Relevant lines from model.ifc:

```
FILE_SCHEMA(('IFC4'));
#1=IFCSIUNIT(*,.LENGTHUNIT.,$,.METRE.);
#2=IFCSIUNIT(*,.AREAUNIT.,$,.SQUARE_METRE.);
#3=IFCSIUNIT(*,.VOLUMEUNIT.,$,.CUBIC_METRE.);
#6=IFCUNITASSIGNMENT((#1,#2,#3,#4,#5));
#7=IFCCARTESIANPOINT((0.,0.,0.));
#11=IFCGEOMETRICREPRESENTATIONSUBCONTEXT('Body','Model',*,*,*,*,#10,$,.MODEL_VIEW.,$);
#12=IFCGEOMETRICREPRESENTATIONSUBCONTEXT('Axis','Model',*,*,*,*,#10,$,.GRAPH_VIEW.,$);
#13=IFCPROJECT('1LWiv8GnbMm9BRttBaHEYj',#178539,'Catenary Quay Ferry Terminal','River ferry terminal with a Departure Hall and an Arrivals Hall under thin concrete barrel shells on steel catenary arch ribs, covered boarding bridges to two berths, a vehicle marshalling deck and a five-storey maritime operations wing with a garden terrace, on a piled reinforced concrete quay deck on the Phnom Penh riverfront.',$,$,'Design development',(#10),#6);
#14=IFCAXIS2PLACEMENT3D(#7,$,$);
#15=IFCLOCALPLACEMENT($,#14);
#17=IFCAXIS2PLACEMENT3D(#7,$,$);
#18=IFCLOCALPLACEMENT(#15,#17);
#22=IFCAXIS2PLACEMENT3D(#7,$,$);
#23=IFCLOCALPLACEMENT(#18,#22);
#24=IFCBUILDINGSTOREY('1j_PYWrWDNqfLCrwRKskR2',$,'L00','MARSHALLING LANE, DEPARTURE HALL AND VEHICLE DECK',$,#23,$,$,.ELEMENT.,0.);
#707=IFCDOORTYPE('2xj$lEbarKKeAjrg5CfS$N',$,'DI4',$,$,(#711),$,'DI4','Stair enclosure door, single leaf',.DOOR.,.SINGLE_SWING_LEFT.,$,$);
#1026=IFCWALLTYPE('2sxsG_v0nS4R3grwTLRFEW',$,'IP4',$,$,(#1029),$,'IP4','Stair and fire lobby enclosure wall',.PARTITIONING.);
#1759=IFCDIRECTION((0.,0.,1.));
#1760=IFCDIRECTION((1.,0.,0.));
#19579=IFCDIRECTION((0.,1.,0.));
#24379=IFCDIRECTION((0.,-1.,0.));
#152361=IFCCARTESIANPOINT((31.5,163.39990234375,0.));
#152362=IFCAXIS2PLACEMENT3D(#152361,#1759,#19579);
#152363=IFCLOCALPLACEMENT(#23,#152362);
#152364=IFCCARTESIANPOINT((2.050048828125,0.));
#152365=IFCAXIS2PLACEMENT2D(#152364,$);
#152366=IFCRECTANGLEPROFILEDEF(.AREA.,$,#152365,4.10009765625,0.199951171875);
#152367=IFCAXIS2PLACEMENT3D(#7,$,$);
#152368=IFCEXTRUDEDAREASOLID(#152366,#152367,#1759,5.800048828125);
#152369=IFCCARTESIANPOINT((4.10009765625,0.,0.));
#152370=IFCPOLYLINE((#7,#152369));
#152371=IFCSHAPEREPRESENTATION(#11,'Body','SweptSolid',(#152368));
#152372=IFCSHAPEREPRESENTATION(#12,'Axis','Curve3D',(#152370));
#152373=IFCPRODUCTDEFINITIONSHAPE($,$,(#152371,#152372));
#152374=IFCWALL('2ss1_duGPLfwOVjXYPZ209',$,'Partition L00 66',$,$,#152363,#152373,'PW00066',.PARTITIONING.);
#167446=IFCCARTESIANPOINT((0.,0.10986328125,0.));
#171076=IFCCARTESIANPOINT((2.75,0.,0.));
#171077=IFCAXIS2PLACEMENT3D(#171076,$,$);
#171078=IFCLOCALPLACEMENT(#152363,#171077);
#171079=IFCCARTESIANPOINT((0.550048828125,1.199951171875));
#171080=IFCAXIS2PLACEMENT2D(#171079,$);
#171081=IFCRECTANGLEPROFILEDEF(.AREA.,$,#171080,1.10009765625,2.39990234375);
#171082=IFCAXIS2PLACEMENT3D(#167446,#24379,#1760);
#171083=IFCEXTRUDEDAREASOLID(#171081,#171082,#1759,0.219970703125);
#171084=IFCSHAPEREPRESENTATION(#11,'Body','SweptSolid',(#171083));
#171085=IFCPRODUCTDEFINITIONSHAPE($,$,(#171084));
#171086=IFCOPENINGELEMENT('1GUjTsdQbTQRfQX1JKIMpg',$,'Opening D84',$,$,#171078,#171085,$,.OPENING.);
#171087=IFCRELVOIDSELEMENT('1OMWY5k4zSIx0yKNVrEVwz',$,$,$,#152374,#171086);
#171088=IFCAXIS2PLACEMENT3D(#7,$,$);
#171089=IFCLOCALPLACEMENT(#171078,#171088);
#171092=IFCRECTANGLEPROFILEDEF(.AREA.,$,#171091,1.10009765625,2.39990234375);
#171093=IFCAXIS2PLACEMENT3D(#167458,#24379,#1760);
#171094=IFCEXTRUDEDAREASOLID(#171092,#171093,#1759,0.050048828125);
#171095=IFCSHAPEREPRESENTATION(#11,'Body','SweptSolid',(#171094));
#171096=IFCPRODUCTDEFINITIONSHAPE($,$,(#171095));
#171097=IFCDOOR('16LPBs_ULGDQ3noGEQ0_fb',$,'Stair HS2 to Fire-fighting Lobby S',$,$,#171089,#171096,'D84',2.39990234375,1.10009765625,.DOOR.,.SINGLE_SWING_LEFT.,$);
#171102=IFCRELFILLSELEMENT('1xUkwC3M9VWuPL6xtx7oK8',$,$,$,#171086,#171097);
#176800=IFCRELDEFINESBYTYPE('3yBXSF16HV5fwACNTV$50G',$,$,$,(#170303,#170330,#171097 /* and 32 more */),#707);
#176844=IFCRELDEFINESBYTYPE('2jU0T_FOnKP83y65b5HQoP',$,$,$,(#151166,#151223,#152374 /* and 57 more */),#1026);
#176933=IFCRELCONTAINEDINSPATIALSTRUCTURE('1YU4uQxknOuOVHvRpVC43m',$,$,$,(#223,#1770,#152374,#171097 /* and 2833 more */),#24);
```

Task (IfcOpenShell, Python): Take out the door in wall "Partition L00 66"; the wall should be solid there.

```python
import ifcopenshell
import ifcopenshell.api.feature
import ifcopenshell.api.root
import ifcopenshell.geom
import ifcopenshell.util.shape

model = ifcopenshell.open("model.ifc")
settings = ifcopenshell.geom.settings()


def volume(element):
    """Net volume in cubic metres, openings subtracted."""
    shape = ifcopenshell.geom.create_shape(settings, element)
    return ifcopenshell.util.shape.get_volume(shape.geometry)


door = model.by_guid("16LPBs_ULGDQ3noGEQ0_fb")
opening = door.FillsVoids[0].RelatingOpeningElement
wall = opening.VoidsElements[0].RelatingBuildingElement
before = volume(wall)

ifcopenshell.api.root.remove_product(model, product=door)
ifcopenshell.api.feature.remove_feature(model, feature=opening)

after = volume(wall)

print(f"wall volume {before:.3f} -> {after:.3f} m3")

model.write("model_v2.ifc")
```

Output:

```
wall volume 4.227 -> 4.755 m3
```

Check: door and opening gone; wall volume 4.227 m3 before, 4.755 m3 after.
